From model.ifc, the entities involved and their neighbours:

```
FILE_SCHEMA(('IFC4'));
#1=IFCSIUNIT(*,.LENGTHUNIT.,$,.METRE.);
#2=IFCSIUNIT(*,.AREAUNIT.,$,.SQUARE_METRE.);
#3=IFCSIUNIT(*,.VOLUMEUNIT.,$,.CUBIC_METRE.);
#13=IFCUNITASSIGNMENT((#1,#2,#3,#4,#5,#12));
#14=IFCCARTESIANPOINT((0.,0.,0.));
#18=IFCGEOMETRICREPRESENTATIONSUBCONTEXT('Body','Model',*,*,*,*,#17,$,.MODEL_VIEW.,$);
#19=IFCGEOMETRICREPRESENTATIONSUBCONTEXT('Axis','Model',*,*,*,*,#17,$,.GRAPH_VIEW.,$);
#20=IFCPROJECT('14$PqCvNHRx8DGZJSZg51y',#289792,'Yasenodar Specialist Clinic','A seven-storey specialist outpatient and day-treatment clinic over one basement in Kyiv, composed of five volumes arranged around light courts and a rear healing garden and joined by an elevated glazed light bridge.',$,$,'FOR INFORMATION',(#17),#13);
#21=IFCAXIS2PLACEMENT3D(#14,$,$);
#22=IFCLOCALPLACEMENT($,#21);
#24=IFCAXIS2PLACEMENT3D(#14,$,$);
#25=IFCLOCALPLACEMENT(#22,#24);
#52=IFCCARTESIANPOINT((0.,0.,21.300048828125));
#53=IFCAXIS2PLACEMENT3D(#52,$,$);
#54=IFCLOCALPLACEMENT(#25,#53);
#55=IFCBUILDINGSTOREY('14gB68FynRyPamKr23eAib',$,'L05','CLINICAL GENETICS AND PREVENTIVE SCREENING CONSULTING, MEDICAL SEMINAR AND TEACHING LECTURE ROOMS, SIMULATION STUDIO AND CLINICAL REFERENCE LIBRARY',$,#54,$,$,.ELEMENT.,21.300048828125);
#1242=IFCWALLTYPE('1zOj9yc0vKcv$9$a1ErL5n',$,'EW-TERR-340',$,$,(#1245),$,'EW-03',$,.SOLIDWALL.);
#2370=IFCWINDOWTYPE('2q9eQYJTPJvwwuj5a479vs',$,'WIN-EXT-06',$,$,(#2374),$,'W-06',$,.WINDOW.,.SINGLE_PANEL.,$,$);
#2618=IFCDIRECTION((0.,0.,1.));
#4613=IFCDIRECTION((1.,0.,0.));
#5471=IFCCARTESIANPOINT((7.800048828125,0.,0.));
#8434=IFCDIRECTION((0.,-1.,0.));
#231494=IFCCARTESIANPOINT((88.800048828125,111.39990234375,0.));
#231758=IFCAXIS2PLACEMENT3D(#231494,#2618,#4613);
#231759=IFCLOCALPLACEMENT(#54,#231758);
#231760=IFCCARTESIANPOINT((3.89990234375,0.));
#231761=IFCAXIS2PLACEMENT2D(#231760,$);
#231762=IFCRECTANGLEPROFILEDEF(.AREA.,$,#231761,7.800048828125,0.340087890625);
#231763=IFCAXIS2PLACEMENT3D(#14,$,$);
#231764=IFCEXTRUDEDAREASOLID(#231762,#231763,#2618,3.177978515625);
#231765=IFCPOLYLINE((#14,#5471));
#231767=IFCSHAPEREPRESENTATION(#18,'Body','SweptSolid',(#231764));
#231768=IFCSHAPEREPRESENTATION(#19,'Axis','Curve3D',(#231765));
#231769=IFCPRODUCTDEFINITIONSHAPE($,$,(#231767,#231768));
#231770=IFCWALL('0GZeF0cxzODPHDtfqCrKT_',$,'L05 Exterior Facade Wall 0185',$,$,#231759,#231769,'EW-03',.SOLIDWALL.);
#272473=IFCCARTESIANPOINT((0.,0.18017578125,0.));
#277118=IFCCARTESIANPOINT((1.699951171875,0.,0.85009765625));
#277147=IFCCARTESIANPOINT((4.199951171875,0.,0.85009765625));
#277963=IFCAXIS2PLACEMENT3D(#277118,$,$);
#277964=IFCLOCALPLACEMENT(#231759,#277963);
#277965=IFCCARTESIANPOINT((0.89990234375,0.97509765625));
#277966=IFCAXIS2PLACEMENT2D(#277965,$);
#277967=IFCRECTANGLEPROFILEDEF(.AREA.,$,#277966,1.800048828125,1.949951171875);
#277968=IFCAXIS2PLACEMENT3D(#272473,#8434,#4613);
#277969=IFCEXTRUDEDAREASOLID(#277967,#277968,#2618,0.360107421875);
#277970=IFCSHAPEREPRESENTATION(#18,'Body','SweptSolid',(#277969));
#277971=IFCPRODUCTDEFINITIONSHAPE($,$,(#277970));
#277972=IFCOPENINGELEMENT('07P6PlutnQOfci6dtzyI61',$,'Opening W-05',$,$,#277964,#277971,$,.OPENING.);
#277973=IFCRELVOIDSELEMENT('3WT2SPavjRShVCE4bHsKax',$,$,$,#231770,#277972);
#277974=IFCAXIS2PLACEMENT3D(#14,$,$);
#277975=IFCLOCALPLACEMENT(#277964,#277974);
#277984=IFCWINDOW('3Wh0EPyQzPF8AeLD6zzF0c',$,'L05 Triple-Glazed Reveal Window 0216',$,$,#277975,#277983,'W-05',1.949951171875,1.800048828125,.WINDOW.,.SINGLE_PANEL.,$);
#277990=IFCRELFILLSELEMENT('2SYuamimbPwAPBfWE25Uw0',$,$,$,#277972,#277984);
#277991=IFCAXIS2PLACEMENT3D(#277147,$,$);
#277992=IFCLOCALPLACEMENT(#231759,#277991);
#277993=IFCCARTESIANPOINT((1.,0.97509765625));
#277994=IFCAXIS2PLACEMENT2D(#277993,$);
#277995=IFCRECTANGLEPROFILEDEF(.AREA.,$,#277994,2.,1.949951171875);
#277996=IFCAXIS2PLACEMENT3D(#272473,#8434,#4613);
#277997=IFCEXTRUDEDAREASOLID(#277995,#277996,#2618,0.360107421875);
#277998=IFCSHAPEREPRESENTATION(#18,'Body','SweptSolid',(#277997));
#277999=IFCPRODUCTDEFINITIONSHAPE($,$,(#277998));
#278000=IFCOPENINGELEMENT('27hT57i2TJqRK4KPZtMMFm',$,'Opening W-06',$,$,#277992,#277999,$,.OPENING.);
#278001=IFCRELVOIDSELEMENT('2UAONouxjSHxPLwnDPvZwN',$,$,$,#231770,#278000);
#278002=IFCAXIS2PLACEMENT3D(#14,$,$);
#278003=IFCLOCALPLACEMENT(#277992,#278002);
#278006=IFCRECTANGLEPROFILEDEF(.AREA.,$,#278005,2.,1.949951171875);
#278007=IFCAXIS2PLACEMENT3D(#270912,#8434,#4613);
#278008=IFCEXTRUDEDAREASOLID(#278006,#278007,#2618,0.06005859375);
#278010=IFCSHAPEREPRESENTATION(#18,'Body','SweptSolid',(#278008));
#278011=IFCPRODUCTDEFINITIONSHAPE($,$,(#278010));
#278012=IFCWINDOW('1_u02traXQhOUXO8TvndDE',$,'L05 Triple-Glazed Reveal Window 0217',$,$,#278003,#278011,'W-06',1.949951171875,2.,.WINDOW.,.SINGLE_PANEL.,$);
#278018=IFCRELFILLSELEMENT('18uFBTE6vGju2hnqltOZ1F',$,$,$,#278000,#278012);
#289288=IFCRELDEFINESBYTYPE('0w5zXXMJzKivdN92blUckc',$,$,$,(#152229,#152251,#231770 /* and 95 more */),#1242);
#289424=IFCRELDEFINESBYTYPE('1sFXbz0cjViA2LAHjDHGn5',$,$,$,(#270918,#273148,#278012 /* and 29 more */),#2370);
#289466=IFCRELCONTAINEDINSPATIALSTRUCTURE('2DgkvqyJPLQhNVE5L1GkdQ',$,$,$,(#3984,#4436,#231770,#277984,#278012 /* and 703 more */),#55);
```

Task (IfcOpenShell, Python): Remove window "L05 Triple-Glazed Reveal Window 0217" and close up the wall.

```python
import ifcopenshell
import ifcopenshell.api.feature
import ifcopenshell.api.root
import ifcopenshell.geom
import ifcopenshell.util.shape

model = ifcopenshell.open("model.ifc")
settings = ifcopenshell.geom.settings()


def volume(element):
    """Net volume in cubic metres, openings subtracted."""
    shape = ifcopenshell.geom.create_shape(settings, element)
    return ifcopenshell.util.shape.get_volume(shape.geometry)


window = model.by_id(278012)
opening = window.FillsVoids[0].RelatingOpeningElement
wall = opening.VoidsElements[0].RelatingBuildingElement
before = volume(wall)

ifcopenshell.api.root.remove_product(model, product=window)
ifcopenshell.api.feature.remove_feature(model, feature=opening)

after = volume(wall)

print(f"wall volume {before:.3f} -> {after:.3f} m3")

model.write("model_updated.ifc")
```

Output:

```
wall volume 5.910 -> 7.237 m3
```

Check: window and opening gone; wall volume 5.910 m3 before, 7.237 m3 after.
